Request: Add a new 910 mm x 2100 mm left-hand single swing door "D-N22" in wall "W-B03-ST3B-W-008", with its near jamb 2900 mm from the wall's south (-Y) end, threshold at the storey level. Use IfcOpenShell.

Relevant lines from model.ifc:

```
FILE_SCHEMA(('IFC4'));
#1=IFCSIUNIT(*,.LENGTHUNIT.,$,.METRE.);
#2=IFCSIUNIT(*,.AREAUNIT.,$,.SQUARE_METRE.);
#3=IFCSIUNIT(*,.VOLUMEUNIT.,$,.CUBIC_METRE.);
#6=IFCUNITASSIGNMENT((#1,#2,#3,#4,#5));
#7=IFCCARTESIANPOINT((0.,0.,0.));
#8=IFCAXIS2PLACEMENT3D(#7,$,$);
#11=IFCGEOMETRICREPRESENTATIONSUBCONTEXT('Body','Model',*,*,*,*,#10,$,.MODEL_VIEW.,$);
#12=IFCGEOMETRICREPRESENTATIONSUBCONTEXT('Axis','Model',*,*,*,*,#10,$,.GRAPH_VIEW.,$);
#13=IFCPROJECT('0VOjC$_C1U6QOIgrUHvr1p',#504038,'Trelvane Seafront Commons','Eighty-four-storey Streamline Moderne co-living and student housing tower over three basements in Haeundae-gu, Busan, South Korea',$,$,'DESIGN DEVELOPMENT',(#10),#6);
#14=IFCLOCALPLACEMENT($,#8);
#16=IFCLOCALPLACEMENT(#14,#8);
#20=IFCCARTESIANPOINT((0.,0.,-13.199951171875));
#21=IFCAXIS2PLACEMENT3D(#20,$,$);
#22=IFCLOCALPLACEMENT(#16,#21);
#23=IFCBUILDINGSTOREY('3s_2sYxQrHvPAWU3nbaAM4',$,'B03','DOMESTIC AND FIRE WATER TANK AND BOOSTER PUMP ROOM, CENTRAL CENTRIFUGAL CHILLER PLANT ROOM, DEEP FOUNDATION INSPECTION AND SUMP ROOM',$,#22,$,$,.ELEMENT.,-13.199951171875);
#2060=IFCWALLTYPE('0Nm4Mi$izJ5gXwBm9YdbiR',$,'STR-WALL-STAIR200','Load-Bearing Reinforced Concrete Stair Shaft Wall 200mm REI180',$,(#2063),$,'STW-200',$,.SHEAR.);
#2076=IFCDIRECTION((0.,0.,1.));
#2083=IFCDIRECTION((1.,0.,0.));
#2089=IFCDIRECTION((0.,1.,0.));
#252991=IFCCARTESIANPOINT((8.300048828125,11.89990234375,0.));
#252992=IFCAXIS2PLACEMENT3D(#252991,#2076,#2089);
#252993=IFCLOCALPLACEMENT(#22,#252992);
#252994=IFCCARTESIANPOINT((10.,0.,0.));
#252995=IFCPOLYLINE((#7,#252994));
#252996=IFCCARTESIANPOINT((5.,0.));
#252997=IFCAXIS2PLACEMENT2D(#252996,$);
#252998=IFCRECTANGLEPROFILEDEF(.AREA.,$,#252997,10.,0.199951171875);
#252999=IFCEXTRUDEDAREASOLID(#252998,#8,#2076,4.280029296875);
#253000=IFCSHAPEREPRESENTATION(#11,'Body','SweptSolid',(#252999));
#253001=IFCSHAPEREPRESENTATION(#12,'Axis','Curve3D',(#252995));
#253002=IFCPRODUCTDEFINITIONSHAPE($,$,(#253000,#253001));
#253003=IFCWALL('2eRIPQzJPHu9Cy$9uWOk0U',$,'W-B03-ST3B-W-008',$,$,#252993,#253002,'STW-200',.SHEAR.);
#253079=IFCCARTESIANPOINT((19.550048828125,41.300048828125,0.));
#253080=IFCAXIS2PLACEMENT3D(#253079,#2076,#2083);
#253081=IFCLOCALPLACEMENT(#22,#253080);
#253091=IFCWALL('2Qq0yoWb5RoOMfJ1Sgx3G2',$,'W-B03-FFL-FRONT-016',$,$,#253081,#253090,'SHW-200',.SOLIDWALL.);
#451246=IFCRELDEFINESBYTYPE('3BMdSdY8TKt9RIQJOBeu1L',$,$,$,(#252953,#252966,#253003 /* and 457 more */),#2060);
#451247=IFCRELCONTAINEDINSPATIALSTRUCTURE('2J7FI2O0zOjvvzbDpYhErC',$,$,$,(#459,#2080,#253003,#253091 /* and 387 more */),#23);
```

```python
import numpy as np
import ifcopenshell
import ifcopenshell.api.feature
import ifcopenshell.api.geometry
import ifcopenshell.api.root
import ifcopenshell.api.spatial
import ifcopenshell.geom
import ifcopenshell.util.element
import ifcopenshell.util.placement
import ifcopenshell.util.representation
import ifcopenshell.util.shape
import ifcopenshell.util.unit

model = ifcopenshell.open("model.ifc")
unit_scale = ifcopenshell.util.unit.calculate_unit_scale(model)
settings = ifcopenshell.geom.settings()


def volume(element):
    """Net volume in cubic metres, openings subtracted."""
    shape = ifcopenshell.geom.create_shape(settings, element)
    return ifcopenshell.util.shape.get_volume(shape.geometry)


wall = model.by_guid("2eRIPQzJPHu9Cy$9uWOk0U")
storey = ifcopenshell.util.element.get_container(wall, ifc_class="IfcBuildingStorey")
context = ifcopenshell.util.representation.get_context(model, "Model", "Body", "MODEL_VIEW")
before = volume(wall)

width, height, from_end, sill = 0.91, 2.1, 2.9, 0.0  # metres

# The wall runs along its own X axis, and the end named is its -X end.
wall_shape = ifcopenshell.geom.create_shape(settings, wall)
x, y, z = ifcopenshell.util.shape.get_vertices(wall_shape.geometry).T
start = x.min() + from_end
face, thickness = float(y.min()), float(y.max() - y.min())
wall_matrix = ifcopenshell.util.placement.get_local_placement(wall.ObjectPlacement)
level = ifcopenshell.util.placement.get_local_placement(storey.ObjectPlacement)[2, 3]


def in_wall(x, y):
    """Placement at x, y metres in the wall's axes, at sill height."""
    matrix = wall_matrix.copy()
    matrix[:, 3] = wall_matrix @ np.array([x / unit_scale, y / unit_scale, 0.0, 1.0])
    matrix[2, 3] = level + sill / unit_scale
    return matrix


# Opening: a box that overshoots both wall faces by 50 mm.
opening = ifcopenshell.api.root.create_entity(model, ifc_class="IfcOpeningElement", predefined_type="OPENING")
box = ifcopenshell.api.geometry.add_wall_representation(
    model, context=context, length=width, height=height, thickness=thickness + 0.1
)
ifcopenshell.api.geometry.assign_representation(model, product=opening, representation=box)
ifcopenshell.api.geometry.edit_object_placement(model, product=opening, matrix=in_wall(start, face - 0.05), is_si=False)
ifcopenshell.api.feature.add_feature(model, feature=opening, element=wall)

door = ifcopenshell.api.root.create_entity(model, ifc_class="IfcDoor", name="D-N22", predefined_type="DOOR")
door.OverallWidth, door.OverallHeight = width / unit_scale, height / unit_scale
door.OperationType = "SINGLE_SWING_LEFT"
body = ifcopenshell.api.geometry.add_door_representation(
    model,
    context=context,
    overall_width=door.OverallWidth,
    overall_height=door.OverallHeight,
    operation_type="SINGLE_SWING_LEFT",
    lining_properties={"LiningDepth": thickness / unit_scale, "ThresholdDepth": thickness / unit_scale},
)
ifcopenshell.api.geometry.assign_representation(model, product=door, representation=body)
ifcopenshell.api.spatial.assign_container(model, products=[door], relating_structure=storey)
ifcopenshell.api.feature.add_filling(model, opening=opening, element=door)

# The lining spans the wall, so the door starts at the wall face.
ifcopenshell.api.geometry.edit_object_placement(model, product=door, matrix=in_wall(start, face), is_si=False)

after = volume(wall)

print(f"wall volume {before:.3f} -> {after:.3f} m3")

model.write("model-out.ifc")
```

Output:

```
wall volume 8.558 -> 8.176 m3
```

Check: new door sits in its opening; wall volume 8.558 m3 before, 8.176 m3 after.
